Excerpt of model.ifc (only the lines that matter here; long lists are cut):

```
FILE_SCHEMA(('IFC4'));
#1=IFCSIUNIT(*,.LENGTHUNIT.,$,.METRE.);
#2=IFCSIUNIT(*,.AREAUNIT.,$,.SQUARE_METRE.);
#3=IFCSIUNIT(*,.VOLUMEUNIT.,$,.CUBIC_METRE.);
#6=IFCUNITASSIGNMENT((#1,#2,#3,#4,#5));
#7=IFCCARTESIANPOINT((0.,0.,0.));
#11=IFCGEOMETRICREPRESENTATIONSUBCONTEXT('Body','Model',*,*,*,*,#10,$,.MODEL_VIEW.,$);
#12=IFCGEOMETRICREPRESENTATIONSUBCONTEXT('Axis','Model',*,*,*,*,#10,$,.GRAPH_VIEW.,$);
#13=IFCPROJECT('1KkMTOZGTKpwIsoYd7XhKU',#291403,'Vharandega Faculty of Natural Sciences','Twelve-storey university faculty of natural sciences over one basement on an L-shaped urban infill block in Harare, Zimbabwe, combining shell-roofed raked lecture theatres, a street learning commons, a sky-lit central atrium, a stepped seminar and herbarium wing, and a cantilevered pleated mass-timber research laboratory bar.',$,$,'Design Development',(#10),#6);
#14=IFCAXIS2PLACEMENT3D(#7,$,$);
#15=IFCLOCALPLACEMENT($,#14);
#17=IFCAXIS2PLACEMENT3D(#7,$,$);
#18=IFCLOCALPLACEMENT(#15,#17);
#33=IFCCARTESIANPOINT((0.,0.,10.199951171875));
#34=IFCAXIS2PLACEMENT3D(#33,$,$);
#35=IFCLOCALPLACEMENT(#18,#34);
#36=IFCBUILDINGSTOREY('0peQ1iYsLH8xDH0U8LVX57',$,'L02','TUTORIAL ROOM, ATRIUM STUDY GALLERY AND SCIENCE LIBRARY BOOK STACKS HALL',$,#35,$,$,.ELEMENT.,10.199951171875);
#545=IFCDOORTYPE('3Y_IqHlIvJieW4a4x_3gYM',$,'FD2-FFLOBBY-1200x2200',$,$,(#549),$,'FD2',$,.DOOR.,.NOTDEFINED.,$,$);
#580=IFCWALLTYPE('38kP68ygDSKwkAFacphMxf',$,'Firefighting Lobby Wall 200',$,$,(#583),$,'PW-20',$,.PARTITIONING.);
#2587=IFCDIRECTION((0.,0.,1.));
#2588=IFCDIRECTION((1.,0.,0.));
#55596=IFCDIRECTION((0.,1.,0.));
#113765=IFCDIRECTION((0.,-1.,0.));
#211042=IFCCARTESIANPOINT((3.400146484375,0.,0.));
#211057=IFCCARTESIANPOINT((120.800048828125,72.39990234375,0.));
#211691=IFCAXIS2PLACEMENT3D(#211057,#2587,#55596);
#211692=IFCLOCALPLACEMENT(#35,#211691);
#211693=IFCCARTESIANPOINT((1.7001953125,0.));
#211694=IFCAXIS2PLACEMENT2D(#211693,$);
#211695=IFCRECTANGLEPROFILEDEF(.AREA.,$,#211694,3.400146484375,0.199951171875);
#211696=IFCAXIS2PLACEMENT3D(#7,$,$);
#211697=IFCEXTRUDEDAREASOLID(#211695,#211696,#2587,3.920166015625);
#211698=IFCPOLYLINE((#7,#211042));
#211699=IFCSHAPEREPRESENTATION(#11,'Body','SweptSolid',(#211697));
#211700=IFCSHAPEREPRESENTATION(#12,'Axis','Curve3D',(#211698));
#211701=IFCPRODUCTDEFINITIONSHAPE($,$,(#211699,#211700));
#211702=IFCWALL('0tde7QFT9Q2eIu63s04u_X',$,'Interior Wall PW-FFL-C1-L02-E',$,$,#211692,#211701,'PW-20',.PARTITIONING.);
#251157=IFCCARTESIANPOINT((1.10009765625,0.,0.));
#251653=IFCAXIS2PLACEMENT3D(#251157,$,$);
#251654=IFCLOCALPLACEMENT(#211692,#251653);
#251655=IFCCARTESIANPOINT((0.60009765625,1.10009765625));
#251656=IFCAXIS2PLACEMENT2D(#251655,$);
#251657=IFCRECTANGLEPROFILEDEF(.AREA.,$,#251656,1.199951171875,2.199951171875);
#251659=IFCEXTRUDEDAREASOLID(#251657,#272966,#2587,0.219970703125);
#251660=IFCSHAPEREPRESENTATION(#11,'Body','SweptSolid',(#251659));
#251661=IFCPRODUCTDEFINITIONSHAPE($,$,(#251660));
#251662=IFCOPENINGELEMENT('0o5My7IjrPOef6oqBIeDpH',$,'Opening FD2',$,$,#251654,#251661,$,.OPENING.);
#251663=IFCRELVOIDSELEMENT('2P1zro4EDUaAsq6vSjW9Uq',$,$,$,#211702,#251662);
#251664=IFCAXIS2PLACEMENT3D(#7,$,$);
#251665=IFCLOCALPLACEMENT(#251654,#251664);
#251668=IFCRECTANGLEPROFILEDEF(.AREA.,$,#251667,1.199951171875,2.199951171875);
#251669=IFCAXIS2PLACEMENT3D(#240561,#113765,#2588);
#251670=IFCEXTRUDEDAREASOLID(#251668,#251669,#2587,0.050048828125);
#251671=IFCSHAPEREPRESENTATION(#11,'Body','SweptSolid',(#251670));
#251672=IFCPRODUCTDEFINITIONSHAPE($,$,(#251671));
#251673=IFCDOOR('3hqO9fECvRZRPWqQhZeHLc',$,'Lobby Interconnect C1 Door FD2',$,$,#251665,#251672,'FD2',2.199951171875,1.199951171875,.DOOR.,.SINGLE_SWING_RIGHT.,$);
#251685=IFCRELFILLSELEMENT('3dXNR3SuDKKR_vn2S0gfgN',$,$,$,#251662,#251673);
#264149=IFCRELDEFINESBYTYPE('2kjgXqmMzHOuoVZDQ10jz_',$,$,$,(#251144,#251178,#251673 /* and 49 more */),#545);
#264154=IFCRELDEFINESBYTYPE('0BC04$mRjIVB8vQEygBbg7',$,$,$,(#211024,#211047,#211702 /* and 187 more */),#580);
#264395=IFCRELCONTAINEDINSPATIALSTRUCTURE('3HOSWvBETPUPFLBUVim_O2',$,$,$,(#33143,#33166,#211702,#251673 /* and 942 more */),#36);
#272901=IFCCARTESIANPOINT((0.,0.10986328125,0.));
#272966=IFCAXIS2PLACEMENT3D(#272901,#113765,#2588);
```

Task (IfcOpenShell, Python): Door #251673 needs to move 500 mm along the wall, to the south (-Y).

```python
import ifcopenshell
import ifcopenshell.api.geometry
import ifcopenshell.util.placement
import ifcopenshell.util.unit

model = ifcopenshell.open("model.ifc")
unit_scale = ifcopenshell.util.unit.calculate_unit_scale(model)

door = model.by_id(251673)
opening = door.FillsVoids[0].RelatingOpeningElement
wall = opening.VoidsElements[0].RelatingBuildingElement

wall_matrix = ifcopenshell.util.placement.get_local_placement(wall.ObjectPlacement)
shift = wall_matrix[:3, 0] * -0.5 / unit_scale
before = ifcopenshell.util.placement.get_local_placement(door.ObjectPlacement)[:3, 3].copy()

# The door is placed relative to its opening, so it follows when the opening moves.
matrix = ifcopenshell.util.placement.get_local_placement(opening.ObjectPlacement)
matrix[:3, 3] += shift
ifcopenshell.api.geometry.edit_object_placement(
    model, product=opening, matrix=matrix, is_si=False, should_transform_children=True
)

after = ifcopenshell.util.placement.get_local_placement(door.ObjectPlacement)[:3, 3]
print("door moved by", (after - before).round(3) + 0.0)

model.write("model_rev.ifc")
```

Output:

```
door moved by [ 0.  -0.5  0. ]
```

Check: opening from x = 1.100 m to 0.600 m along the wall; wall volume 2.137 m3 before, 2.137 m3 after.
